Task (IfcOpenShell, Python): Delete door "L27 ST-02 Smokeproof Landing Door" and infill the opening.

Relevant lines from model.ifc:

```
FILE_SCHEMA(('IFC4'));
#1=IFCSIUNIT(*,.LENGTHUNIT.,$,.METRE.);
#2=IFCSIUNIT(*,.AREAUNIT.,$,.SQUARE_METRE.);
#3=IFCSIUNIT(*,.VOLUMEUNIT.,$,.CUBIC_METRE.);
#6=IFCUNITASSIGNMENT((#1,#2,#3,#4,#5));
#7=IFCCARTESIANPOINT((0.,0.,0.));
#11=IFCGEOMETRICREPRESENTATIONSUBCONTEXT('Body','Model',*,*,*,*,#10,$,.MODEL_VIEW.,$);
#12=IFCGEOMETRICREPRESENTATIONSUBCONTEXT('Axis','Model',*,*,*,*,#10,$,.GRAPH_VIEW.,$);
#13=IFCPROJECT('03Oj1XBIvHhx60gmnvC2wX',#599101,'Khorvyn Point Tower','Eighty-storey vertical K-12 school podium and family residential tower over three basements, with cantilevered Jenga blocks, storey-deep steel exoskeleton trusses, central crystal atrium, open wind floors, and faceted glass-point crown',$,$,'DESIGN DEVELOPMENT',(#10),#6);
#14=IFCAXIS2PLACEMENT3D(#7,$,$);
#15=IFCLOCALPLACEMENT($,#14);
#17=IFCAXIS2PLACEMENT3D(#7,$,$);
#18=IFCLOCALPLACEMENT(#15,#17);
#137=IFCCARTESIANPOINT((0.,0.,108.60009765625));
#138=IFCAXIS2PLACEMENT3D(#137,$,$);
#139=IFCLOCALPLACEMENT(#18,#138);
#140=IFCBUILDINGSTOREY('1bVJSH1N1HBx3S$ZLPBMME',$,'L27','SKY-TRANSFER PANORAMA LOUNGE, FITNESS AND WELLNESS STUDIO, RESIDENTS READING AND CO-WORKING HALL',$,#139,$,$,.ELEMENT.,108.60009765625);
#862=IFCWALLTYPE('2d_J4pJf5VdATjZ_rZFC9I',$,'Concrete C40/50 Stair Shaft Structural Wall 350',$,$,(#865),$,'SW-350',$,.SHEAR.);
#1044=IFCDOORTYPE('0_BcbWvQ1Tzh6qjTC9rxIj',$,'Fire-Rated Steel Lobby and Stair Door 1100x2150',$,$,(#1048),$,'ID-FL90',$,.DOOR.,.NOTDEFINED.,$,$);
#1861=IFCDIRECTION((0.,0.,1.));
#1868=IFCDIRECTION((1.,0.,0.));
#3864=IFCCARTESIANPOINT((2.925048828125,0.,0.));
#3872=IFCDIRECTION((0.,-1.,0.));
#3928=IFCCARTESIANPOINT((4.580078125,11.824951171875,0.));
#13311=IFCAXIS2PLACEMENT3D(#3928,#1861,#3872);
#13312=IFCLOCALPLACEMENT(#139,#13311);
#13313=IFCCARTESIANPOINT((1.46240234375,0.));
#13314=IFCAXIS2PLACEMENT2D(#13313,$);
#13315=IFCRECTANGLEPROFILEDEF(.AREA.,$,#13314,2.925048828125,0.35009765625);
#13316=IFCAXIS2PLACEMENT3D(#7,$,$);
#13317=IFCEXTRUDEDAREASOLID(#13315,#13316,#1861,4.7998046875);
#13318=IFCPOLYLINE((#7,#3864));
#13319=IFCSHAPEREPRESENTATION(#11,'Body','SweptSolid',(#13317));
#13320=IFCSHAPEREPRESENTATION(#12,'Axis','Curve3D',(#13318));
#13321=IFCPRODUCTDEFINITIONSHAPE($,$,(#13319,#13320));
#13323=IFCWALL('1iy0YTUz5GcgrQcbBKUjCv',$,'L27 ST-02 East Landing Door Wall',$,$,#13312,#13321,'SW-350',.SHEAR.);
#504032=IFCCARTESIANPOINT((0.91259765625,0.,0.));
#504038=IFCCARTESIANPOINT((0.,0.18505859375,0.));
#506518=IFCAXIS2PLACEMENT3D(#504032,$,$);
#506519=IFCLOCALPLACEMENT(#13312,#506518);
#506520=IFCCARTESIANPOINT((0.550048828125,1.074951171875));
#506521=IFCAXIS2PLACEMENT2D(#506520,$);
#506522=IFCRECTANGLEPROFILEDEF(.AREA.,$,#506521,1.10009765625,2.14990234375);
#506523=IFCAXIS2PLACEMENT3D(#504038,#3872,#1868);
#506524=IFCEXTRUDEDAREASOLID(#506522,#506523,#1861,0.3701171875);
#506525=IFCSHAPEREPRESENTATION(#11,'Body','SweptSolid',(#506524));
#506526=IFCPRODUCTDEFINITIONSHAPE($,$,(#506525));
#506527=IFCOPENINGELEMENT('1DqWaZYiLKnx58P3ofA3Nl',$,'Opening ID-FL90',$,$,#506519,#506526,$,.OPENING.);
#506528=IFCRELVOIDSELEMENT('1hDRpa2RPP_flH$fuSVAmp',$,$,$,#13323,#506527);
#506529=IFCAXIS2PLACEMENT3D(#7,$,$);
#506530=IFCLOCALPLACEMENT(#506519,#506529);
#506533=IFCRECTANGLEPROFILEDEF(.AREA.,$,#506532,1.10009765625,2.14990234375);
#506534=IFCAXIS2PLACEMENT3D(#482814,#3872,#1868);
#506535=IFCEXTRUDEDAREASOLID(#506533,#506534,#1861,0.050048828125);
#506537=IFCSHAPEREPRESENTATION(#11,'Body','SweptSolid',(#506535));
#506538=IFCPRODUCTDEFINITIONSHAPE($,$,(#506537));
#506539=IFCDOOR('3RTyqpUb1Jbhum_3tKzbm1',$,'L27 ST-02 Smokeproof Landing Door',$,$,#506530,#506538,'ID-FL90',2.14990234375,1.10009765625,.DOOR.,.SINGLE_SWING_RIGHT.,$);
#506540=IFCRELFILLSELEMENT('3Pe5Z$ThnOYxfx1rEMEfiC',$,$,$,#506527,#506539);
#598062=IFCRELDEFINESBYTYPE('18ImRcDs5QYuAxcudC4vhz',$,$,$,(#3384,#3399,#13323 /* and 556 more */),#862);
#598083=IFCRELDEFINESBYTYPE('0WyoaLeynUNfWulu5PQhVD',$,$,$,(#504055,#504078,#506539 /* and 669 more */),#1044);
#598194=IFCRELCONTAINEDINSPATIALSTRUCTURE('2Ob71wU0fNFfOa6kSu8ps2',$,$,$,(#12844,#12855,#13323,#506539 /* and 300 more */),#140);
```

```python
import ifcopenshell
import ifcopenshell.api.feature
import ifcopenshell.api.root
import ifcopenshell.geom
import ifcopenshell.util.shape

model = ifcopenshell.open("model.ifc")
settings = ifcopenshell.geom.settings()


def volume(element):
    """Net volume in cubic metres, openings subtracted."""
    shape = ifcopenshell.geom.create_shape(settings, element)
    return ifcopenshell.util.shape.get_volume(shape.geometry)


door = model.by_guid("3RTyqpUb1Jbhum_3tKzbm1")
opening = door.FillsVoids[0].RelatingOpeningElement
wall = opening.VoidsElements[0].RelatingBuildingElement
before = volume(wall)

ifcopenshell.api.root.remove_product(model, product=door)
ifcopenshell.api.feature.remove_feature(model, feature=opening)

after = volume(wall)

print(f"wall volume {before:.3f} -> {after:.3f} m3")

model.write("model_rev.ifc")
```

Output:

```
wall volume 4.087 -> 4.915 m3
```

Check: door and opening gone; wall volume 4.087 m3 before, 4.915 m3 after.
